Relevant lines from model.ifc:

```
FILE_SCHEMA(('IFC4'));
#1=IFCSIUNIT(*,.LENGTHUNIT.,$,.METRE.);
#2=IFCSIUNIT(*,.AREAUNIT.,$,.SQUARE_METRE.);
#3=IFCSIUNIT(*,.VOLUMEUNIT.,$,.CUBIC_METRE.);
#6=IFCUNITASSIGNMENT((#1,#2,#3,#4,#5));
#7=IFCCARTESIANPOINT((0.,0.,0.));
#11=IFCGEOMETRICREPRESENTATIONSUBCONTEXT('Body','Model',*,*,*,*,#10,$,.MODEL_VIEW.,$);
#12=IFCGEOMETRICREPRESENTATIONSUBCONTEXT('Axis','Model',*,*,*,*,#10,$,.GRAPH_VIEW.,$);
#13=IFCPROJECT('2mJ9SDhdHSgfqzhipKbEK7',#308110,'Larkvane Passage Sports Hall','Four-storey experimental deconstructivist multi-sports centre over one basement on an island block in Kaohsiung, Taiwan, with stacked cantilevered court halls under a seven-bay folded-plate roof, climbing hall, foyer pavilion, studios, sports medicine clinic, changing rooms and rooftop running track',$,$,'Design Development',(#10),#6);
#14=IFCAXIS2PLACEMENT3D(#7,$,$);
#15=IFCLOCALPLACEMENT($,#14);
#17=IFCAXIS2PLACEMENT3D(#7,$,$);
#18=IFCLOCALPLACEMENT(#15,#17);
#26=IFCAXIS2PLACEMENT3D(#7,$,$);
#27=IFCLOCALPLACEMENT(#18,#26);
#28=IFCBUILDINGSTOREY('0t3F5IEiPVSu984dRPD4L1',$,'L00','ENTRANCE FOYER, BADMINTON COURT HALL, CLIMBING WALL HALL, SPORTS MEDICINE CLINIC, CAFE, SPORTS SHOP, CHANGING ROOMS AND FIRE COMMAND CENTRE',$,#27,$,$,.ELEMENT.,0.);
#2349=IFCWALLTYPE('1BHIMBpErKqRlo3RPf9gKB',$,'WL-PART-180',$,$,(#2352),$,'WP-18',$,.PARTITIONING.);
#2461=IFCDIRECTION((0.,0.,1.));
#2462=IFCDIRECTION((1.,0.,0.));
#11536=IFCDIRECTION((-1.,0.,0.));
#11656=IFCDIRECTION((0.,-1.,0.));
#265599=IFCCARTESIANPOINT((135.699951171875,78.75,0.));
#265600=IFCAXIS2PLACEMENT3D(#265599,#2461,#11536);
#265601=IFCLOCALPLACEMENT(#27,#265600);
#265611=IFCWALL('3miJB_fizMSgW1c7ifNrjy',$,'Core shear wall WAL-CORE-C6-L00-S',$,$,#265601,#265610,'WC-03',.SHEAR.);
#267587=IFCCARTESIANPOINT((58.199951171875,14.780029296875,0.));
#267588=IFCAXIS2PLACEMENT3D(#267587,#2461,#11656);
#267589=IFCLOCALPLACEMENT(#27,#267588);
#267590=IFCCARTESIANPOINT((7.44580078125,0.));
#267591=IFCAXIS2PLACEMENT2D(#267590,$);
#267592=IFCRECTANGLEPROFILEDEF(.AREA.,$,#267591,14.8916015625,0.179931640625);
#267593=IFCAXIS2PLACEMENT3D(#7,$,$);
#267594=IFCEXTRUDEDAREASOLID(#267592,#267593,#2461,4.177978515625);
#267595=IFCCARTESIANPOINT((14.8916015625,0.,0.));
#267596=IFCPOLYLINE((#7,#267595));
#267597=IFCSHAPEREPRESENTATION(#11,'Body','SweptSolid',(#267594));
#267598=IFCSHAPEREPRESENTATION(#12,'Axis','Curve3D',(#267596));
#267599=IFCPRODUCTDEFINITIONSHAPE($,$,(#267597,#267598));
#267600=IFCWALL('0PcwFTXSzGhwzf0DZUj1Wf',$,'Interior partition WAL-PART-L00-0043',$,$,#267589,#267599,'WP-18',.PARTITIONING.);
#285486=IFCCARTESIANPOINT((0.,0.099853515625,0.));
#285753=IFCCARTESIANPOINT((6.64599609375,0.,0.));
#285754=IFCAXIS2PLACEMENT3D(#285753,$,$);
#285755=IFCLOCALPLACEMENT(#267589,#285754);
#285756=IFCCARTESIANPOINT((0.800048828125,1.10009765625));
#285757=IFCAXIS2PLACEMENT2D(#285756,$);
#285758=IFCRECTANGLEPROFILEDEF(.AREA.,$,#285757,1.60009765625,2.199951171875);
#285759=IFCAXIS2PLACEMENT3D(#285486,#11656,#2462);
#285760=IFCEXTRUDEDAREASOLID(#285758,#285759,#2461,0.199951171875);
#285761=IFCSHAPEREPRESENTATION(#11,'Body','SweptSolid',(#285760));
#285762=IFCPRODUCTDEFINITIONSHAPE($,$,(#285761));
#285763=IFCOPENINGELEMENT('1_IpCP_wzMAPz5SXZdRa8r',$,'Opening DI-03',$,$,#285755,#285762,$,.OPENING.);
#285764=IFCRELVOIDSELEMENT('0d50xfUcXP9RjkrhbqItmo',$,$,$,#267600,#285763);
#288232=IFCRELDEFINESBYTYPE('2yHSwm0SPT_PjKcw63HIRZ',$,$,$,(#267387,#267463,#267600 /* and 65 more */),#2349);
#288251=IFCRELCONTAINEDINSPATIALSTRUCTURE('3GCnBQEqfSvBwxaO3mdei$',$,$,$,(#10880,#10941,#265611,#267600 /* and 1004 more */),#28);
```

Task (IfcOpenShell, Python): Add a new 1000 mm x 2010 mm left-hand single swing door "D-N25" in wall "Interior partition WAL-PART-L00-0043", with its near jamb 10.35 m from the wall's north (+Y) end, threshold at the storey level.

```python
import numpy as np
import ifcopenshell
import ifcopenshell.api.feature
import ifcopenshell.api.geometry
import ifcopenshell.api.root
import ifcopenshell.api.spatial
import ifcopenshell.geom
import ifcopenshell.util.element
import ifcopenshell.util.placement
import ifcopenshell.util.representation
import ifcopenshell.util.shape
import ifcopenshell.util.unit

model = ifcopenshell.open("model.ifc")
unit_scale = ifcopenshell.util.unit.calculate_unit_scale(model)
settings = ifcopenshell.geom.settings()


def volume(element):
    """Net volume in cubic metres, openings subtracted."""
    shape = ifcopenshell.geom.create_shape(settings, element)
    return ifcopenshell.util.shape.get_volume(shape.geometry)


wall = model.by_guid("0PcwFTXSzGhwzf0DZUj1Wf")
storey = ifcopenshell.util.element.get_container(wall, ifc_class="IfcBuildingStorey")
context = ifcopenshell.util.representation.get_context(model, "Model", "Body", "MODEL_VIEW")
before = volume(wall)

width, height, from_end, sill = 1, 2.01, 10.35, 0.0  # metres

# The wall runs along its own X axis, and the end named is its -X end.
wall_shape = ifcopenshell.geom.create_shape(settings, wall)
x, y, z = ifcopenshell.util.shape.get_vertices(wall_shape.geometry).T
start = x.min() + from_end
face, thickness = float(y.min()), float(y.max() - y.min())
wall_matrix = ifcopenshell.util.placement.get_local_placement(wall.ObjectPlacement)
level = ifcopenshell.util.placement.get_local_placement(storey.ObjectPlacement)[2, 3]


def in_wall(x, y):
    """Placement at x, y metres in the wall's axes, at sill height."""
    matrix = wall_matrix.copy()
    matrix[:, 3] = wall_matrix @ np.array([x / unit_scale, y / unit_scale, 0.0, 1.0])
    matrix[2, 3] = level + sill / unit_scale
    return matrix


# Opening: a box that overshoots both wall faces by 50 mm.
opening = ifcopenshell.api.root.create_entity(model, ifc_class="IfcOpeningElement", predefined_type="OPENING")
box = ifcopenshell.api.geometry.add_wall_representation(
    model, context=context, length=width, height=height, thickness=thickness + 0.1
)
ifcopenshell.api.geometry.assign_representation(model, product=opening, representation=box)
ifcopenshell.api.geometry.edit_object_placement(model, product=opening, matrix=in_wall(start, face - 0.05), is_si=False)
ifcopenshell.api.feature.add_feature(model, feature=opening, element=wall)

door = ifcopenshell.api.root.create_entity(model, ifc_class="IfcDoor", name="D-N25", predefined_type="DOOR")
door.OverallWidth, door.OverallHeight = width / unit_scale, height / unit_scale
door.OperationType = "SINGLE_SWING_LEFT"
body = ifcopenshell.api.geometry.add_door_representation(
    model,
    context=context,
    overall_width=door.OverallWidth,
    overall_height=door.OverallHeight,
    operation_type="SINGLE_SWING_LEFT",
    lining_properties={"LiningDepth": thickness / unit_scale, "ThresholdDepth": thickness / unit_scale},
)
ifcopenshell.api.geometry.assign_representation(model, product=door, representation=body)
ifcopenshell.api.spatial.assign_container(model, products=[door], relating_structure=storey)
ifcopenshell.api.feature.add_filling(model, opening=opening, element=door)

# The lining spans the wall, so the door starts at the wall face.
ifcopenshell.api.geometry.edit_object_placement(model, product=door, matrix=in_wall(start, face), is_si=False)

after = volume(wall)

print(f"wall volume {before:.3f} -> {after:.3f} m3")

model.write("model_edited.ifc")
```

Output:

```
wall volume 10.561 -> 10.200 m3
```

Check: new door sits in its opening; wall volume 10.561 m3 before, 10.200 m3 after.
